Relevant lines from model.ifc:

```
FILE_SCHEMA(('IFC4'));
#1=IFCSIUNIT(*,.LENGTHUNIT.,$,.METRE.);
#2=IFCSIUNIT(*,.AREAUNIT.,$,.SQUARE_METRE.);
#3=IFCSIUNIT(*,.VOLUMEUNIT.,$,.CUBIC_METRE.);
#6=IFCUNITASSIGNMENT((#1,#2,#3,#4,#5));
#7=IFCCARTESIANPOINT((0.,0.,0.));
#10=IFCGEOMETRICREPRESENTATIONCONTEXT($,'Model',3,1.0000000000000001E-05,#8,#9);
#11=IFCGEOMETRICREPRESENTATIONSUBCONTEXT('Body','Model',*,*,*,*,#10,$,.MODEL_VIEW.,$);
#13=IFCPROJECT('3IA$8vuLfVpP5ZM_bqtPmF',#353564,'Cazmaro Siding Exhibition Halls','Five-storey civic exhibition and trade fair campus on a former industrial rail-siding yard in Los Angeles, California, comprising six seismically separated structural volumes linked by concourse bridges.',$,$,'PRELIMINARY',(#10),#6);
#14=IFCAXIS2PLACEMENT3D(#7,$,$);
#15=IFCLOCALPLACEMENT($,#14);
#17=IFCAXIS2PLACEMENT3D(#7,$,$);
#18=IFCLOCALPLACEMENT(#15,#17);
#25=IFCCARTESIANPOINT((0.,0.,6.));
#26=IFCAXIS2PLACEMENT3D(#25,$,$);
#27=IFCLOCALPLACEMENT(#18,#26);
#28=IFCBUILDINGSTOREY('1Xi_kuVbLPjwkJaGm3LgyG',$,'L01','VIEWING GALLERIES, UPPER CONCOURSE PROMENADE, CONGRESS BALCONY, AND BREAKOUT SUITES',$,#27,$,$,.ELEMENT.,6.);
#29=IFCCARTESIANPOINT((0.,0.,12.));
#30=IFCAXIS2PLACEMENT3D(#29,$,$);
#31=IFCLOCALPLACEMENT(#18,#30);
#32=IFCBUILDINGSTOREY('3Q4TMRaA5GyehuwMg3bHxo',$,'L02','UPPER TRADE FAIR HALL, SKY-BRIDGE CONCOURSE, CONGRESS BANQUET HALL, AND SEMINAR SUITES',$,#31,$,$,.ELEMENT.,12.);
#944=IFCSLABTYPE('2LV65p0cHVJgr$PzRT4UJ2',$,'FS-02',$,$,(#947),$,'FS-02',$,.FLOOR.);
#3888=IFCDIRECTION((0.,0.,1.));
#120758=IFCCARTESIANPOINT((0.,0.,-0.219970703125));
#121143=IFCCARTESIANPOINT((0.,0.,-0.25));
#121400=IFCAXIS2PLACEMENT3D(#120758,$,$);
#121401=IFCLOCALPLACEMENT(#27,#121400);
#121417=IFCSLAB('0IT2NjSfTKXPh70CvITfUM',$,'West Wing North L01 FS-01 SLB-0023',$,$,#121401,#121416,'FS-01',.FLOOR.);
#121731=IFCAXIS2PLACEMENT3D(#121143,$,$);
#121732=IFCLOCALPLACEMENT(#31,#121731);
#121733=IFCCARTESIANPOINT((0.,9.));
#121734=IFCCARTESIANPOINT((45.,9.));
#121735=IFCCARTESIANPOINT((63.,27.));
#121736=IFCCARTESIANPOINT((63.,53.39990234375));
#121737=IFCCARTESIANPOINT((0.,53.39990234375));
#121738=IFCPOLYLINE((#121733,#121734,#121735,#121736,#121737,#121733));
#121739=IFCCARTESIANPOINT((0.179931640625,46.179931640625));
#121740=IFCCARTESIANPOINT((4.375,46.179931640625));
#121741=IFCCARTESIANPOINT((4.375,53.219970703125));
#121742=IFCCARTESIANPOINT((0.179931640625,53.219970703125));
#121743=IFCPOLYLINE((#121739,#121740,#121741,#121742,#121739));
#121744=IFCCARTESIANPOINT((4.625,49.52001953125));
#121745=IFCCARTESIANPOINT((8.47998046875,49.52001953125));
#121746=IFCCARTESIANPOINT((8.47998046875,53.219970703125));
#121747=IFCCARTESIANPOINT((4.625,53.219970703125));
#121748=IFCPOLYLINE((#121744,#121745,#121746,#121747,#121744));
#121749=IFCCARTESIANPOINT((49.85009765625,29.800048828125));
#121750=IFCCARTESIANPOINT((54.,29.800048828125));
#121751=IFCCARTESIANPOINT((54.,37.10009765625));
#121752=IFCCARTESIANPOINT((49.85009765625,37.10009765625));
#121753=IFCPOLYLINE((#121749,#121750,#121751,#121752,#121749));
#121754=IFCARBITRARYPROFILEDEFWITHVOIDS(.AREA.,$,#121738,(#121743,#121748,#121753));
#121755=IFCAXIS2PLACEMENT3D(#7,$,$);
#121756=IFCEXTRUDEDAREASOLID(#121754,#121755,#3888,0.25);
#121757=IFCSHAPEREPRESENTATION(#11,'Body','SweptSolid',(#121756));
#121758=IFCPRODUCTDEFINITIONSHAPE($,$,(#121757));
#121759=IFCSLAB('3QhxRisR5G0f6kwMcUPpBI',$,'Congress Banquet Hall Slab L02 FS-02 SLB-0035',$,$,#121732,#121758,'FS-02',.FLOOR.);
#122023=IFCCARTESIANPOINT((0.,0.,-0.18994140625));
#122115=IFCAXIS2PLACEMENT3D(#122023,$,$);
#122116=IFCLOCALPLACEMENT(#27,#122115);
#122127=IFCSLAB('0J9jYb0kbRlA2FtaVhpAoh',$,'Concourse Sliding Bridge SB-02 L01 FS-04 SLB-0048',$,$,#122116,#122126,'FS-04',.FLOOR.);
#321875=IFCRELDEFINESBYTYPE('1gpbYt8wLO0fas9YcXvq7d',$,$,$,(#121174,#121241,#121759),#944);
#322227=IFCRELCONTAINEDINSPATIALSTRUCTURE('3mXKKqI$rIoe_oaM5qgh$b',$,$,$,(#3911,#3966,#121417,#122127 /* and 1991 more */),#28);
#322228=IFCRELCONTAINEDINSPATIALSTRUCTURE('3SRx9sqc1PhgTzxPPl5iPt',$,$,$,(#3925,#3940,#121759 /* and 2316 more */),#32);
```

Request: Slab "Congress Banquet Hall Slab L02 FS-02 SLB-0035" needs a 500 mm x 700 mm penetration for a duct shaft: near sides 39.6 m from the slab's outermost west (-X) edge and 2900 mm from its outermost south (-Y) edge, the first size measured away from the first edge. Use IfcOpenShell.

```python
import numpy as np
import ifcopenshell
import ifcopenshell.api.feature
import ifcopenshell.api.geometry
import ifcopenshell.api.root
import ifcopenshell.geom
import ifcopenshell.util.placement
import ifcopenshell.util.representation
import ifcopenshell.util.shape
import ifcopenshell.util.unit

model = ifcopenshell.open("model.ifc")
unit_scale = ifcopenshell.util.unit.calculate_unit_scale(model)
settings = ifcopenshell.geom.settings()


def volume(element):
    """Net volume in cubic metres, openings subtracted."""
    shape = ifcopenshell.geom.create_shape(settings, element)
    return ifcopenshell.util.shape.get_volume(shape.geometry)


slab = model.by_id(121759)
before = volume(slab)

# Extent in the slab's own axes, in metres. The edges named are its -X and -Y sides.
slab_shape = ifcopenshell.geom.create_shape(settings, slab)
vertices = ifcopenshell.util.shape.get_vertices(slab_shape.geometry)
x_min, y_min, bottom = vertices.min(axis=0)
top = vertices[:, 2].max()

opening = ifcopenshell.api.root.create_entity(model, ifc_class="IfcOpeningElement", name="Duct shaft opening", predefined_type="OPENING")
context = ifcopenshell.util.representation.get_context(model, "Model", "Body", "MODEL_VIEW")
width, depth = 0.5, 0.7
outline = [(0.0, 0.0), (width, 0.0), (width, depth), (0.0, depth), (0.0, 0.0)]
# Overshoot both faces by 50 mm so the cut is clean.
shape = ifcopenshell.api.geometry.add_slab_representation(
    model, context=context, depth=top - bottom + 0.1, polyline=outline
)
ifcopenshell.api.geometry.assign_representation(model, product=opening, representation=shape)

matrix = ifcopenshell.util.placement.get_local_placement(slab.ObjectPlacement)
matrix[:, 3] = matrix @ np.append(np.array([x_min + 39.6, y_min + 2.9, bottom - 0.05]) / unit_scale, 1.0)
ifcopenshell.api.geometry.edit_object_placement(model, product=opening, matrix=matrix, is_si=False)
ifcopenshell.api.feature.add_feature(model, feature=opening, element=slab)

after = volume(slab)

print(f"slab volume {before:.3f} -> {after:.3f} m3")

model.write("model_updated.ifc")
```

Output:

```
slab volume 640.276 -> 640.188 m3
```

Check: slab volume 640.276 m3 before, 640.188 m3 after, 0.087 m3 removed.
